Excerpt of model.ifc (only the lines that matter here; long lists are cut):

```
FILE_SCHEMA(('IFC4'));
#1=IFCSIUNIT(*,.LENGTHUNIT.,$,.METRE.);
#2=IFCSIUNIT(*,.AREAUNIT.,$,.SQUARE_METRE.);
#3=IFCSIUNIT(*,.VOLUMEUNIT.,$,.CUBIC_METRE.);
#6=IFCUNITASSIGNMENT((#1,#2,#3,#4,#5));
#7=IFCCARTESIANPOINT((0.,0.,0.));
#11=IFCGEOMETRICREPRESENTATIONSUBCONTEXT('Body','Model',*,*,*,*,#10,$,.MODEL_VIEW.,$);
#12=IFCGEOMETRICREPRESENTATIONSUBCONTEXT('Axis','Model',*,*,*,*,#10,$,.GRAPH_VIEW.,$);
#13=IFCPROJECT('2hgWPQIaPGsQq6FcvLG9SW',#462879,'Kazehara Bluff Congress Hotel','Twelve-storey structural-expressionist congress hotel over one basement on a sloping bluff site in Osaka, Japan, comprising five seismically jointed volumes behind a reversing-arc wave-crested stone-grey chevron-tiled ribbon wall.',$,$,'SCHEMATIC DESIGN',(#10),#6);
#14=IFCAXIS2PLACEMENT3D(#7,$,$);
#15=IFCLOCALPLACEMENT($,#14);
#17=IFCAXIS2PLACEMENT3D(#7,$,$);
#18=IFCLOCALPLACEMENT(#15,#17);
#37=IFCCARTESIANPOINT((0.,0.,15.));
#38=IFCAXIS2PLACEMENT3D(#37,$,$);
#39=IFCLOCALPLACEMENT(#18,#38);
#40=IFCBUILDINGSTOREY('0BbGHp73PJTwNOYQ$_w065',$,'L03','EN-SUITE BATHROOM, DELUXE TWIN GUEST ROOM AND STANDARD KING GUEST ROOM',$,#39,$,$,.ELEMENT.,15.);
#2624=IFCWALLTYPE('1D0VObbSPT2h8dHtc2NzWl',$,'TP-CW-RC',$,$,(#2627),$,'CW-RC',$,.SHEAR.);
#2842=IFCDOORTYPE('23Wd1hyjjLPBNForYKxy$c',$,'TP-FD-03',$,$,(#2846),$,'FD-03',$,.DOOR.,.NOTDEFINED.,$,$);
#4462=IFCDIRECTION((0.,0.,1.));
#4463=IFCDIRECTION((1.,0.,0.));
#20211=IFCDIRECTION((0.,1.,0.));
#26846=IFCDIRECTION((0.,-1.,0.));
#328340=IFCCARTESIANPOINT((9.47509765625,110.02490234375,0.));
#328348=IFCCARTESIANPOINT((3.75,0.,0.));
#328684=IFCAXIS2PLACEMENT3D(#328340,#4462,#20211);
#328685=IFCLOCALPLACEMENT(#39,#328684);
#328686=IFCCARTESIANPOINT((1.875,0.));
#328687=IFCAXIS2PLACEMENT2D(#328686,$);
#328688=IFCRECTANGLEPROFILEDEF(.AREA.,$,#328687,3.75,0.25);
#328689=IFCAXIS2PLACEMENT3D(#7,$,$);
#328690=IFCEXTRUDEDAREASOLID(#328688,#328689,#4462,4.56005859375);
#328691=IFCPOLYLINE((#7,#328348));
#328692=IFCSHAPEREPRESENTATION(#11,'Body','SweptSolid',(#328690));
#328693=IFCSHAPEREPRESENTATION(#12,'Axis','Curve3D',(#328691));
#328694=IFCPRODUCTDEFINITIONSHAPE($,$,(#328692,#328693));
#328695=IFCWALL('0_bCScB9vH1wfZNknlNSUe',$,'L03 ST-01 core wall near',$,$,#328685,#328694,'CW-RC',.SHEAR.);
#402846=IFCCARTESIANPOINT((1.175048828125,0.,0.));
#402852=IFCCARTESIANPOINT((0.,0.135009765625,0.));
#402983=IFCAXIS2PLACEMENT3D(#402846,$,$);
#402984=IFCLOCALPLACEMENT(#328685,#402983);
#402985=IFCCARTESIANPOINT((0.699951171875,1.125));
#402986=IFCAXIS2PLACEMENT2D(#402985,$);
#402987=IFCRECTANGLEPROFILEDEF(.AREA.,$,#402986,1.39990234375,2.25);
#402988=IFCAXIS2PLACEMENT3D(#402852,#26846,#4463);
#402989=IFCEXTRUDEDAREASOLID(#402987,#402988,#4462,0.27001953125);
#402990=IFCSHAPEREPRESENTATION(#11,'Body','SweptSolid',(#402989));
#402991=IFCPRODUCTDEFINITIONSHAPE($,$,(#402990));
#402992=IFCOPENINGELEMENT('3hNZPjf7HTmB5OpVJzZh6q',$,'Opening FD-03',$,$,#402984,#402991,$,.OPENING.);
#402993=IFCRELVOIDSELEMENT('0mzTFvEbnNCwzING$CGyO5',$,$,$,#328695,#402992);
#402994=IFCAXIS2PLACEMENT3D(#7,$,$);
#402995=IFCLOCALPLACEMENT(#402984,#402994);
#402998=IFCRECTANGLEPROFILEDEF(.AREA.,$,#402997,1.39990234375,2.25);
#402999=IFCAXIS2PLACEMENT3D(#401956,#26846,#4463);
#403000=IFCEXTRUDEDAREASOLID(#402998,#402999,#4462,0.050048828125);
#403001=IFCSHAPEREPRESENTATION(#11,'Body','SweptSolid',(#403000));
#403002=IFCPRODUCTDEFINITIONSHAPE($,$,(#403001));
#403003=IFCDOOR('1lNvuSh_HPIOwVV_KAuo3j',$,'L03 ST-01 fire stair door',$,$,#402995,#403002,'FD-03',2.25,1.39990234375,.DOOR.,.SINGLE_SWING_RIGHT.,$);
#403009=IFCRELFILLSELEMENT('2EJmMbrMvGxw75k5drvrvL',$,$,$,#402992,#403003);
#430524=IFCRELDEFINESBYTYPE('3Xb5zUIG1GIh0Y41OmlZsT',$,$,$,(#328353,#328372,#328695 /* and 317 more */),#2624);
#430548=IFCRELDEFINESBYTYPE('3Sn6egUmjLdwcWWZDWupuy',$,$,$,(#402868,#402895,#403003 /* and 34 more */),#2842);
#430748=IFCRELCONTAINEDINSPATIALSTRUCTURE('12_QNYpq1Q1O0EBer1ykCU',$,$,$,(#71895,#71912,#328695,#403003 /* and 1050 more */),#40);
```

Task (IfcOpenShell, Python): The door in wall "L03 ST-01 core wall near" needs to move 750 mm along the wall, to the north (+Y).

```python
import ifcopenshell
import ifcopenshell.api.geometry
import ifcopenshell.util.placement
import ifcopenshell.util.unit

model = ifcopenshell.open("model.ifc")
unit_scale = ifcopenshell.util.unit.calculate_unit_scale(model)

door = model.by_guid("1lNvuSh_HPIOwVV_KAuo3j")
opening = door.FillsVoids[0].RelatingOpeningElement
wall = opening.VoidsElements[0].RelatingBuildingElement

wall_matrix = ifcopenshell.util.placement.get_local_placement(wall.ObjectPlacement)
shift = wall_matrix[:3, 0] * 0.75 / unit_scale
before = ifcopenshell.util.placement.get_local_placement(door.ObjectPlacement)[:3, 3].copy()

# The door is placed relative to its opening, so it follows when the opening moves.
matrix = ifcopenshell.util.placement.get_local_placement(opening.ObjectPlacement)
matrix[:3, 3] += shift
ifcopenshell.api.geometry.edit_object_placement(
    model, product=opening, matrix=matrix, is_si=False, should_transform_children=True
)

after = ifcopenshell.util.placement.get_local_placement(door.ObjectPlacement)[:3, 3]
print("door moved by", (after - before).round(3) + 0.0)

model.write("model_rev.ifc")
```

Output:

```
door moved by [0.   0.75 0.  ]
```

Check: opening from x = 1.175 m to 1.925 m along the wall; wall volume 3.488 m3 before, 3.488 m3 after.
